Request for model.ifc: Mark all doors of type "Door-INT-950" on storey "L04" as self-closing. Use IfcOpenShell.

First a look at what the model holds.

```python
import ifcopenshell
import ifcopenshell.util.element

model = ifcopenshell.open("model.ifc")
print(model.schema)
storey = next(s for s in model.by_type("IfcBuildingStorey") if s.Name == "L04")
doors = [e for e in ifcopenshell.util.element.get_decomposition(storey) if e.is_a("IfcDoor")]
seen = {}
for e in doors:
    element_type = ifcopenshell.util.element.get_type(e)
    key = (element_type.Name if element_type != e and element_type else None, ifcopenshell.util.element.get_pset(e, "Pset_DoorCommon", "SelfClosing"))
    seen[key] = seen.get(key, 0) + 1
for (name, value), count in sorted(seen.items(), key=str):
    print(count, "x", name, "|", value)
```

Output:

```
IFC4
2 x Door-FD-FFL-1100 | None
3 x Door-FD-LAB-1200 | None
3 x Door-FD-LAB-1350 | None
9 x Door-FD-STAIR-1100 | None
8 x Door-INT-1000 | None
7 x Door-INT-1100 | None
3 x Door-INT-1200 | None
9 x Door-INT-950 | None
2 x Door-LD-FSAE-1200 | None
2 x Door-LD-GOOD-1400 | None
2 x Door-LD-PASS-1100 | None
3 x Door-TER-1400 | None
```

```python
import ifcopenshell
import ifcopenshell.api.pset
import ifcopenshell.util.element

model = ifcopenshell.open("model.ifc")

storey = next(s for s in model.by_type("IfcBuildingStorey") if s.Name == "L04")
doors = [e for e in ifcopenshell.util.element.get_decomposition(storey) if e.is_a("IfcDoor")]

count = 0
for e in doors:
    element_type = ifcopenshell.util.element.get_type(e)
    if element_type in (None, e) or element_type.Name != "Door-INT-950":
        continue
    # add_pset returns the element's existing set when there is one.
    pset = ifcopenshell.api.pset.add_pset(model, product=e, name="Pset_DoorCommon")
    ifcopenshell.api.pset.edit_pset(model, pset=pset, properties={"SelfClosing": True})
    count += 1

print(count, "doors updated")

model.write("model_updated.ifc")
```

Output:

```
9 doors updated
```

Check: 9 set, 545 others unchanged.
